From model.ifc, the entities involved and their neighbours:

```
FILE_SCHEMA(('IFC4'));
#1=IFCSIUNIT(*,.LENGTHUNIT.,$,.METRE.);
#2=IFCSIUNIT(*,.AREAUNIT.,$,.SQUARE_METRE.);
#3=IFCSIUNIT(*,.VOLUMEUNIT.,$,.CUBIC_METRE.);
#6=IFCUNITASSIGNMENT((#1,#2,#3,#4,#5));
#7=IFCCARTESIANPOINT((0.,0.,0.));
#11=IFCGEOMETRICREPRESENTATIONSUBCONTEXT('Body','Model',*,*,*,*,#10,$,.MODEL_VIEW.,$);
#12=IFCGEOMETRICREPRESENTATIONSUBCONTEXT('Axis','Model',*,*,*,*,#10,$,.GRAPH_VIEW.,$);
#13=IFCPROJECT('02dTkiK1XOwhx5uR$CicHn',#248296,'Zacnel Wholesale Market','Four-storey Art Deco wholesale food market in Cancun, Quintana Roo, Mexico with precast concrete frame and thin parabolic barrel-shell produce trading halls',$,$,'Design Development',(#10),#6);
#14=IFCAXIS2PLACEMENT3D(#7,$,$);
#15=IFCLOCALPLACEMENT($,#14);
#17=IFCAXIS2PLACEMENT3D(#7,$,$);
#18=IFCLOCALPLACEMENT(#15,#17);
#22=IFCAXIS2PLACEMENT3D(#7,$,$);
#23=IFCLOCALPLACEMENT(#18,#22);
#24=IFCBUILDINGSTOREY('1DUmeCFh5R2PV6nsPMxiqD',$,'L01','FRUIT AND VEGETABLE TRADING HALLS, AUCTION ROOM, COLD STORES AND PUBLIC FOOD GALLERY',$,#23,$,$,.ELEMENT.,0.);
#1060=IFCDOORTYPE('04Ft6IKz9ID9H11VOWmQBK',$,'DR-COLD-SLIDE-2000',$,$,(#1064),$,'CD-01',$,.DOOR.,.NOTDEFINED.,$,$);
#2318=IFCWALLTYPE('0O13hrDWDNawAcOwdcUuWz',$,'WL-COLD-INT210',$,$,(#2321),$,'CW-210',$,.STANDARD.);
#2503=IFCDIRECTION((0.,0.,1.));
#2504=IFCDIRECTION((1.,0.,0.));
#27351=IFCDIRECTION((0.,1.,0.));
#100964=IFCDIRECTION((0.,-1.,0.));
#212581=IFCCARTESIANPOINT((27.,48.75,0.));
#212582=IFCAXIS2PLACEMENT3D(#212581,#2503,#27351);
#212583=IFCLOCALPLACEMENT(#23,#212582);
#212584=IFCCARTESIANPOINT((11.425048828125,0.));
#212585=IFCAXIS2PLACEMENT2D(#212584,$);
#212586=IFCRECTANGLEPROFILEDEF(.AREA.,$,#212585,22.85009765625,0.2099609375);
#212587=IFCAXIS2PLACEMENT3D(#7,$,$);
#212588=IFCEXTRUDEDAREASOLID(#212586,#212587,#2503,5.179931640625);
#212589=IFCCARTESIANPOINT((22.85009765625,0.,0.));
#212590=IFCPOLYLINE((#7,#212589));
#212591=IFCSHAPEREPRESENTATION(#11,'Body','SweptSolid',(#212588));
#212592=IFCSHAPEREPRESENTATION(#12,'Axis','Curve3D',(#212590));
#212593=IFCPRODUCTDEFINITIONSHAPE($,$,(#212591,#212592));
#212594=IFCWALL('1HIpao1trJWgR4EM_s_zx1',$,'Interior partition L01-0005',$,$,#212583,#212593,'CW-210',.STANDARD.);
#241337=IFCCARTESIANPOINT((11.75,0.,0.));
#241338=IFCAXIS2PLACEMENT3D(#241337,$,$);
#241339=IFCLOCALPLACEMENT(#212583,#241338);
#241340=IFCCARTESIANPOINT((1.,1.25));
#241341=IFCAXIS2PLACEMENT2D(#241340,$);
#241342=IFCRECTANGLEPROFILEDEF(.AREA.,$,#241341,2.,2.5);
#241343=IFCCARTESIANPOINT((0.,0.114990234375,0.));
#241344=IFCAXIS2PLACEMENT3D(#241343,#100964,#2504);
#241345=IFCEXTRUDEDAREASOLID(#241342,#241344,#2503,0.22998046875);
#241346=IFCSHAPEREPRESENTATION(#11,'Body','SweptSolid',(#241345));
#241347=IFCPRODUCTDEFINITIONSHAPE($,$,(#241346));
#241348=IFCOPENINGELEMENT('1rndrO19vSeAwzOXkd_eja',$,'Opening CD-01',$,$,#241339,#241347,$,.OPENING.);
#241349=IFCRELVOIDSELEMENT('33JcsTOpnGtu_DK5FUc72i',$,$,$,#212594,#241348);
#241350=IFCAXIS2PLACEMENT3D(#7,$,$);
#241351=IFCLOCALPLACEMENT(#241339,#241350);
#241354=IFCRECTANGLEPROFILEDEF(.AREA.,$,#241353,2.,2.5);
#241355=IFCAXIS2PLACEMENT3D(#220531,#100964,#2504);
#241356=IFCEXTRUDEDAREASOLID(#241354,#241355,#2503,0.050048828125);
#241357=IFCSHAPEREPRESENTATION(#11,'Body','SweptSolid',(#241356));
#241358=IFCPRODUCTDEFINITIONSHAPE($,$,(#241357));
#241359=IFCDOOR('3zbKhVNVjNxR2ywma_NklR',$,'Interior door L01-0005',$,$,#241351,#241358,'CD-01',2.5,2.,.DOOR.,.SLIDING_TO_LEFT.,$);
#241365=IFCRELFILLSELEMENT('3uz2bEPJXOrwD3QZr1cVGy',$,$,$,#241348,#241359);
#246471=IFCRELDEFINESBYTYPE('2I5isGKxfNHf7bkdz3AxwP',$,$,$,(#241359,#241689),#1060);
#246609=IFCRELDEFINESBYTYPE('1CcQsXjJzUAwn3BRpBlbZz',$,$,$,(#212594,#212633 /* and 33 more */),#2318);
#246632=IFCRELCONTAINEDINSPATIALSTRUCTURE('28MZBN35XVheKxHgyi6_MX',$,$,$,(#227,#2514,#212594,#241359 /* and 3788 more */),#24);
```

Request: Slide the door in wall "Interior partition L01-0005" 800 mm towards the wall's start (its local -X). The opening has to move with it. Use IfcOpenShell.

```python
import ifcopenshell
import ifcopenshell.api.geometry
import ifcopenshell.util.placement

model = ifcopenshell.open("model.ifc")

door = model.by_guid("3zbKhVNVjNxR2ywma_NklR")
opening = door.FillsVoids[0].RelatingOpeningElement
wall = opening.VoidsElements[0].RelatingBuildingElement

wall_matrix = ifcopenshell.util.placement.get_local_placement(wall.ObjectPlacement)
shift = wall_matrix[:3, 0] * -0.8
before = ifcopenshell.util.placement.get_local_placement(door.ObjectPlacement)[:3, 3].copy()

# The door is placed relative to its opening, so it follows when the opening moves.
matrix = ifcopenshell.util.placement.get_local_placement(opening.ObjectPlacement)
matrix[:3, 3] += shift
ifcopenshell.api.geometry.edit_object_placement(
    model, product=opening, matrix=matrix, is_si=False, should_transform_children=True
)

after = ifcopenshell.util.placement.get_local_placement(door.ObjectPlacement)[:3, 3]
print("door moved by", (after - before).round(3) + 0.0)

model.write("model-out.ifc")
```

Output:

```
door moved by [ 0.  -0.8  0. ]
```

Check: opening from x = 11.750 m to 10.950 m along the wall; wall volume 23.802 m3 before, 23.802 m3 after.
